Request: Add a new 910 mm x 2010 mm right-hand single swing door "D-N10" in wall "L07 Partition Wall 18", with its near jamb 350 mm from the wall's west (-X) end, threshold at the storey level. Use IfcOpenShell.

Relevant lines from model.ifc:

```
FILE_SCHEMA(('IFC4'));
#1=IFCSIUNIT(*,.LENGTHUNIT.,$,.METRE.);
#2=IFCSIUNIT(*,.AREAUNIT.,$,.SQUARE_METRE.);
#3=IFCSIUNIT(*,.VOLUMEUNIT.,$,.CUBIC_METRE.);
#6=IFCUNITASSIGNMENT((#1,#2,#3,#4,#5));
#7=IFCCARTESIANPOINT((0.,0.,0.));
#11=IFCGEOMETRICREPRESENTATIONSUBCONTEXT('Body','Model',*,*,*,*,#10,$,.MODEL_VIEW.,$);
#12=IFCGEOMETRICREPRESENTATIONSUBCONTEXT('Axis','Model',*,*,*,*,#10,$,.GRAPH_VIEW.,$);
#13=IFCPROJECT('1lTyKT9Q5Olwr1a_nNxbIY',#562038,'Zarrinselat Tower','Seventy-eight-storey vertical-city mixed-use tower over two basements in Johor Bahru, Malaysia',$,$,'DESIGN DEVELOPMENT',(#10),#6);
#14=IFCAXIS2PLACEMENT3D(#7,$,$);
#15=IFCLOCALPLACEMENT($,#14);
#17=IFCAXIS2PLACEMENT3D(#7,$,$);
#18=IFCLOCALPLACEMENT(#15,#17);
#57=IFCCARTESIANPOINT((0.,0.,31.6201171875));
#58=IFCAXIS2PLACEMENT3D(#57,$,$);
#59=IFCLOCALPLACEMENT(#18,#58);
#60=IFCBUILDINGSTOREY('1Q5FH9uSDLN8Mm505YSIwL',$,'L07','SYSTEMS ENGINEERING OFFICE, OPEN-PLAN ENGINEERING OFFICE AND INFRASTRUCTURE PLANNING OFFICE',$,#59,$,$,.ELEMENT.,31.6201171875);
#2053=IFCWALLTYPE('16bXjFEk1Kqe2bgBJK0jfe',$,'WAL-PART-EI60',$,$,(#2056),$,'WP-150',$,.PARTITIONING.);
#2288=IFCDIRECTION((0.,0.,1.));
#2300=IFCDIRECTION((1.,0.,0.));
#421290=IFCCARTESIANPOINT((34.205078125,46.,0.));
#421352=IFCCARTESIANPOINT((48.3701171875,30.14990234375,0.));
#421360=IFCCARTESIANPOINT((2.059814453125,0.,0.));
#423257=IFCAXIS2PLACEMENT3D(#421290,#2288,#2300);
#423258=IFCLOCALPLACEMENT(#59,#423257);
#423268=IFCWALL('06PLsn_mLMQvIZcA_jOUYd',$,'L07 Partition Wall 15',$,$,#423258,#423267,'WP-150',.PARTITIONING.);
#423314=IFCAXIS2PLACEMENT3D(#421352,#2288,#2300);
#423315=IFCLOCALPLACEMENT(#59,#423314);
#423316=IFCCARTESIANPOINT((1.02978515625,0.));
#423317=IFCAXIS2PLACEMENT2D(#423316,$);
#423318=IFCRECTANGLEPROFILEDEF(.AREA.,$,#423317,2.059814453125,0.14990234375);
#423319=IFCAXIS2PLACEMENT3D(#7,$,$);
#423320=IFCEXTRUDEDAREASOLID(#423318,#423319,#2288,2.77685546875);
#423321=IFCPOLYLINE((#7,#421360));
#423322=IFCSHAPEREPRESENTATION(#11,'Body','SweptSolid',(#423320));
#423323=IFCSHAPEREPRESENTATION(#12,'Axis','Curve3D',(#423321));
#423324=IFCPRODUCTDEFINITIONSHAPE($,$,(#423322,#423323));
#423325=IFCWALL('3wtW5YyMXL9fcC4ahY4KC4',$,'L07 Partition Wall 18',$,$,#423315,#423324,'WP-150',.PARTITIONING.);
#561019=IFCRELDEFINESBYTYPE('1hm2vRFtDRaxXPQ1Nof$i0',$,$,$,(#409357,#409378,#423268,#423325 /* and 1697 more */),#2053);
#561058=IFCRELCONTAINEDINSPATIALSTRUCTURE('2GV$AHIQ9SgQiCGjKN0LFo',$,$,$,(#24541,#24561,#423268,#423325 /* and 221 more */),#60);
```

```python
import numpy as np
import ifcopenshell
import ifcopenshell.api.feature
import ifcopenshell.api.geometry
import ifcopenshell.api.root
import ifcopenshell.api.spatial
import ifcopenshell.geom
import ifcopenshell.util.element
import ifcopenshell.util.placement
import ifcopenshell.util.representation
import ifcopenshell.util.shape
import ifcopenshell.util.unit

model = ifcopenshell.open("model.ifc")
unit_scale = ifcopenshell.util.unit.calculate_unit_scale(model)
settings = ifcopenshell.geom.settings()


def volume(element):
    """Net volume in cubic metres, openings subtracted."""
    shape = ifcopenshell.geom.create_shape(settings, element)
    return ifcopenshell.util.shape.get_volume(shape.geometry)


wall = model.by_guid("3wtW5YyMXL9fcC4ahY4KC4")
storey = ifcopenshell.util.element.get_container(wall, ifc_class="IfcBuildingStorey")
context = ifcopenshell.util.representation.get_context(model, "Model", "Body", "MODEL_VIEW")
before = volume(wall)

width, height, from_end, sill = 0.91, 2.01, 0.35, 0.0  # metres

# The wall runs along its own X axis, and the end named is its -X end.
wall_shape = ifcopenshell.geom.create_shape(settings, wall)
x, y, z = ifcopenshell.util.shape.get_vertices(wall_shape.geometry).T
start = x.min() + from_end
face, thickness = float(y.min()), float(y.max() - y.min())
wall_matrix = ifcopenshell.util.placement.get_local_placement(wall.ObjectPlacement)
level = ifcopenshell.util.placement.get_local_placement(storey.ObjectPlacement)[2, 3]


def in_wall(x, y):
    """Placement at x, y metres in the wall's axes, at sill height."""
    matrix = wall_matrix.copy()
    matrix[:, 3] = wall_matrix @ np.array([x / unit_scale, y / unit_scale, 0.0, 1.0])
    matrix[2, 3] = level + sill / unit_scale
    return matrix


# Opening: a box that overshoots both wall faces by 50 mm.
opening = ifcopenshell.api.root.create_entity(model, ifc_class="IfcOpeningElement", predefined_type="OPENING")
box = ifcopenshell.api.geometry.add_wall_representation(
    model, context=context, length=width, height=height, thickness=thickness + 0.1
)
ifcopenshell.api.geometry.assign_representation(model, product=opening, representation=box)
ifcopenshell.api.geometry.edit_object_placement(model, product=opening, matrix=in_wall(start, face - 0.05), is_si=False)
ifcopenshell.api.feature.add_feature(model, feature=opening, element=wall)

door = ifcopenshell.api.root.create_entity(model, ifc_class="IfcDoor", name="D-N10", predefined_type="DOOR")
door.OverallWidth, door.OverallHeight = width / unit_scale, height / unit_scale
door.OperationType = "SINGLE_SWING_RIGHT"
body = ifcopenshell.api.geometry.add_door_representation(
    model,
    context=context,
    overall_width=door.OverallWidth,
    overall_height=door.OverallHeight,
    operation_type="SINGLE_SWING_RIGHT",
    lining_properties={"LiningDepth": thickness / unit_scale, "ThresholdDepth": thickness / unit_scale},
)
ifcopenshell.api.geometry.assign_representation(model, product=door, representation=body)
ifcopenshell.api.spatial.assign_container(model, products=[door], relating_structure=storey)
ifcopenshell.api.feature.add_filling(model, opening=opening, element=door)

# The lining spans the wall, so the door starts at the wall face.
ifcopenshell.api.geometry.edit_object_placement(model, product=door, matrix=in_wall(start, face), is_si=False)

after = volume(wall)

print(f"wall volume {before:.3f} -> {after:.3f} m3")

model.write("model_edited.ifc")
```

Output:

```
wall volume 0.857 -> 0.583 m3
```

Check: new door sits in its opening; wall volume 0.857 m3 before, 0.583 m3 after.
